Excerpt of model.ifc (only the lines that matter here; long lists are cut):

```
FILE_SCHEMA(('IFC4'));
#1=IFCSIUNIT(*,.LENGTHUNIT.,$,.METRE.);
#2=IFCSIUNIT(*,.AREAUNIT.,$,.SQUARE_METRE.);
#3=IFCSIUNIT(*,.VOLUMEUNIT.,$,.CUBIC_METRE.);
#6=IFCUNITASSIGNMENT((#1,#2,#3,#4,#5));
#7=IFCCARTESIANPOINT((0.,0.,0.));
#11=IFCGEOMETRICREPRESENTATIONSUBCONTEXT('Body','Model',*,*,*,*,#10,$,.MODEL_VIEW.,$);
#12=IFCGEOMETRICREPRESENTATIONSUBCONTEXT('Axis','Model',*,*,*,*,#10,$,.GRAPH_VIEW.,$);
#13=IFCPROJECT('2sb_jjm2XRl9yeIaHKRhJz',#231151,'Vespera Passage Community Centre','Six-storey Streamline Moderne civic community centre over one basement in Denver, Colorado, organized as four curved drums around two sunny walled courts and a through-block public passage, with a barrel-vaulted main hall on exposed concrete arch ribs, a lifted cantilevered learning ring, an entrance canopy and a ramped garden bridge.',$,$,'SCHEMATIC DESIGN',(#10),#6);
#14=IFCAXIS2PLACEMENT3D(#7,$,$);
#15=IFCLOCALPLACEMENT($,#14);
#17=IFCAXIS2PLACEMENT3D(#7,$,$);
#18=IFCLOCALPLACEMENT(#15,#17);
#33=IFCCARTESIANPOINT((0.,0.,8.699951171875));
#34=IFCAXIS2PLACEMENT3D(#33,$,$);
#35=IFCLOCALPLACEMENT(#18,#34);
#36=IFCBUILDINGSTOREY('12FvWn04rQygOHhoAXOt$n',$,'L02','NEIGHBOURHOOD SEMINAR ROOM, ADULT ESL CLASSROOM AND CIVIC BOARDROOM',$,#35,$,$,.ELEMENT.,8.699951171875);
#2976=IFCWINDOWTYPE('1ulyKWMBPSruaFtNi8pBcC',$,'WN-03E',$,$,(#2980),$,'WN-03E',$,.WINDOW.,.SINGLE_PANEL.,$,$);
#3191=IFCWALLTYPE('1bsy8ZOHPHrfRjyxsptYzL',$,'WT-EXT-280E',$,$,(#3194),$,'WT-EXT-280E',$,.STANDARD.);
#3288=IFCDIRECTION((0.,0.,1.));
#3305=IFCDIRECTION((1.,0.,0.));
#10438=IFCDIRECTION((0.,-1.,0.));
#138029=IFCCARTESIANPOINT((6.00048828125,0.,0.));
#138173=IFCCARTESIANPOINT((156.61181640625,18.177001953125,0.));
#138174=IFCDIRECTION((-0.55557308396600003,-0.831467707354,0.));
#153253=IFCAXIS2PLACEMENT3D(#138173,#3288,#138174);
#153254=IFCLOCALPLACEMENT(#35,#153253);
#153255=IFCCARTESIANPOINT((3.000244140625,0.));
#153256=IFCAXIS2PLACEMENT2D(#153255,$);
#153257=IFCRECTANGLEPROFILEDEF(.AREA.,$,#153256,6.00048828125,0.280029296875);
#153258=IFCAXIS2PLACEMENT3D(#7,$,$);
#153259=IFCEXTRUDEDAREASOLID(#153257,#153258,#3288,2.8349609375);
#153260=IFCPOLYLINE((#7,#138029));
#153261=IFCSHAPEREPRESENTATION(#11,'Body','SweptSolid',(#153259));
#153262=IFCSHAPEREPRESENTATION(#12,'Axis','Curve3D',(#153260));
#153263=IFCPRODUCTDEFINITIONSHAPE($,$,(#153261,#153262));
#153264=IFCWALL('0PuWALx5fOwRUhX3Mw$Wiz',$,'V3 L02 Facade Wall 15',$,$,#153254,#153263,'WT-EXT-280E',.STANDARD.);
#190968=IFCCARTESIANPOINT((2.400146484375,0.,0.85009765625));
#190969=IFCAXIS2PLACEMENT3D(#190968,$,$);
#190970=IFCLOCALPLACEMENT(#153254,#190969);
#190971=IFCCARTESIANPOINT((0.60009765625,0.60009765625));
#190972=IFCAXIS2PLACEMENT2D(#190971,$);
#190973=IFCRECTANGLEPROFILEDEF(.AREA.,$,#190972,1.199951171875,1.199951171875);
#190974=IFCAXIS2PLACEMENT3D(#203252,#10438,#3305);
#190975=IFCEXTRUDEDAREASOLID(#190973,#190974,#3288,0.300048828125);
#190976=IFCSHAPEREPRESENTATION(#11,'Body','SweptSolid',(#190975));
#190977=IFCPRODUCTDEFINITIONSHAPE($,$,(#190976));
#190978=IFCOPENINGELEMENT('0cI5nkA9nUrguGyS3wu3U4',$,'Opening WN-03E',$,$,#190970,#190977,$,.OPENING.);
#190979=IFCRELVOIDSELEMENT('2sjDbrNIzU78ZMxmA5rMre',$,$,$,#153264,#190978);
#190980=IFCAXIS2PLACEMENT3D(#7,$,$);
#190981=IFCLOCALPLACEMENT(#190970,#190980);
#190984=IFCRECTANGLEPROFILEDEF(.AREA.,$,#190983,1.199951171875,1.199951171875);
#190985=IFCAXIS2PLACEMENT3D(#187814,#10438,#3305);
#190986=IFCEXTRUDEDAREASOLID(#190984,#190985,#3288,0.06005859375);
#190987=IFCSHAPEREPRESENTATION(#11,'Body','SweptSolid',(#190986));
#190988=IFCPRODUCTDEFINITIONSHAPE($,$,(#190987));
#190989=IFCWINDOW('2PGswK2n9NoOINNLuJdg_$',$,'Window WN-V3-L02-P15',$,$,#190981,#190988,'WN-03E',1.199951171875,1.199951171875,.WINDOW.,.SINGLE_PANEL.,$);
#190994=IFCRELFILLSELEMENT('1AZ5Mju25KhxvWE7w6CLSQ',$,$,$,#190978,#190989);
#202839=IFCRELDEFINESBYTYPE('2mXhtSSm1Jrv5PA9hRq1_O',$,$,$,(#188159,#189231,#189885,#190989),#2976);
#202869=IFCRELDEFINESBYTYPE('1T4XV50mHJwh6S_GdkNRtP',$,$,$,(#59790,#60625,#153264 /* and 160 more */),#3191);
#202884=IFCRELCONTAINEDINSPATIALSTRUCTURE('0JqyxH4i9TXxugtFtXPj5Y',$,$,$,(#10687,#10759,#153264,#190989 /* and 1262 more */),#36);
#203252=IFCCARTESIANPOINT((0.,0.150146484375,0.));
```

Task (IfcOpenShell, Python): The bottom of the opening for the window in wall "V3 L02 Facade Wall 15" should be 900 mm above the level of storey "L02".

```python
import numpy as np
import ifcopenshell
import ifcopenshell.api.geometry
import ifcopenshell.geom
import ifcopenshell.util.element
import ifcopenshell.util.placement
import ifcopenshell.util.shape
import ifcopenshell.util.unit

model = ifcopenshell.open("model.ifc")
unit_scale = ifcopenshell.util.unit.calculate_unit_scale(model)

window = model.by_guid("2PGswK2n9NoOINNLuJdg_$")
opening = window.FillsVoids[0].RelatingOpeningElement
storey = ifcopenshell.util.element.get_container(window, ifc_class="IfcBuildingStorey")
level = ifcopenshell.util.placement.get_local_placement(storey.ObjectPlacement)[2, 3]

# The opening's origin need not be at the sill, so measure its lowest point.
shape = ifcopenshell.geom.create_shape(ifcopenshell.geom.settings(), opening)
bottom = ifcopenshell.util.shape.get_shape_bottom_elevation(shape, shape.geometry) / unit_scale
dz = level + 0.9 - bottom

shift = np.array([0.0, 0.0, dz])
# The window is placed relative to its opening, so it follows when the opening moves.
matrix = ifcopenshell.util.placement.get_local_placement(opening.ObjectPlacement)
matrix[:3, 3] += shift
ifcopenshell.api.geometry.edit_object_placement(
    model, product=opening, matrix=matrix, is_si=False, should_transform_children=True
)

print(f"moved by {dz * unit_scale:+.3f} m")

model.write("model_rev.ifc")
```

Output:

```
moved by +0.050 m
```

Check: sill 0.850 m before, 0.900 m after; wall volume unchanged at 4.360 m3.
